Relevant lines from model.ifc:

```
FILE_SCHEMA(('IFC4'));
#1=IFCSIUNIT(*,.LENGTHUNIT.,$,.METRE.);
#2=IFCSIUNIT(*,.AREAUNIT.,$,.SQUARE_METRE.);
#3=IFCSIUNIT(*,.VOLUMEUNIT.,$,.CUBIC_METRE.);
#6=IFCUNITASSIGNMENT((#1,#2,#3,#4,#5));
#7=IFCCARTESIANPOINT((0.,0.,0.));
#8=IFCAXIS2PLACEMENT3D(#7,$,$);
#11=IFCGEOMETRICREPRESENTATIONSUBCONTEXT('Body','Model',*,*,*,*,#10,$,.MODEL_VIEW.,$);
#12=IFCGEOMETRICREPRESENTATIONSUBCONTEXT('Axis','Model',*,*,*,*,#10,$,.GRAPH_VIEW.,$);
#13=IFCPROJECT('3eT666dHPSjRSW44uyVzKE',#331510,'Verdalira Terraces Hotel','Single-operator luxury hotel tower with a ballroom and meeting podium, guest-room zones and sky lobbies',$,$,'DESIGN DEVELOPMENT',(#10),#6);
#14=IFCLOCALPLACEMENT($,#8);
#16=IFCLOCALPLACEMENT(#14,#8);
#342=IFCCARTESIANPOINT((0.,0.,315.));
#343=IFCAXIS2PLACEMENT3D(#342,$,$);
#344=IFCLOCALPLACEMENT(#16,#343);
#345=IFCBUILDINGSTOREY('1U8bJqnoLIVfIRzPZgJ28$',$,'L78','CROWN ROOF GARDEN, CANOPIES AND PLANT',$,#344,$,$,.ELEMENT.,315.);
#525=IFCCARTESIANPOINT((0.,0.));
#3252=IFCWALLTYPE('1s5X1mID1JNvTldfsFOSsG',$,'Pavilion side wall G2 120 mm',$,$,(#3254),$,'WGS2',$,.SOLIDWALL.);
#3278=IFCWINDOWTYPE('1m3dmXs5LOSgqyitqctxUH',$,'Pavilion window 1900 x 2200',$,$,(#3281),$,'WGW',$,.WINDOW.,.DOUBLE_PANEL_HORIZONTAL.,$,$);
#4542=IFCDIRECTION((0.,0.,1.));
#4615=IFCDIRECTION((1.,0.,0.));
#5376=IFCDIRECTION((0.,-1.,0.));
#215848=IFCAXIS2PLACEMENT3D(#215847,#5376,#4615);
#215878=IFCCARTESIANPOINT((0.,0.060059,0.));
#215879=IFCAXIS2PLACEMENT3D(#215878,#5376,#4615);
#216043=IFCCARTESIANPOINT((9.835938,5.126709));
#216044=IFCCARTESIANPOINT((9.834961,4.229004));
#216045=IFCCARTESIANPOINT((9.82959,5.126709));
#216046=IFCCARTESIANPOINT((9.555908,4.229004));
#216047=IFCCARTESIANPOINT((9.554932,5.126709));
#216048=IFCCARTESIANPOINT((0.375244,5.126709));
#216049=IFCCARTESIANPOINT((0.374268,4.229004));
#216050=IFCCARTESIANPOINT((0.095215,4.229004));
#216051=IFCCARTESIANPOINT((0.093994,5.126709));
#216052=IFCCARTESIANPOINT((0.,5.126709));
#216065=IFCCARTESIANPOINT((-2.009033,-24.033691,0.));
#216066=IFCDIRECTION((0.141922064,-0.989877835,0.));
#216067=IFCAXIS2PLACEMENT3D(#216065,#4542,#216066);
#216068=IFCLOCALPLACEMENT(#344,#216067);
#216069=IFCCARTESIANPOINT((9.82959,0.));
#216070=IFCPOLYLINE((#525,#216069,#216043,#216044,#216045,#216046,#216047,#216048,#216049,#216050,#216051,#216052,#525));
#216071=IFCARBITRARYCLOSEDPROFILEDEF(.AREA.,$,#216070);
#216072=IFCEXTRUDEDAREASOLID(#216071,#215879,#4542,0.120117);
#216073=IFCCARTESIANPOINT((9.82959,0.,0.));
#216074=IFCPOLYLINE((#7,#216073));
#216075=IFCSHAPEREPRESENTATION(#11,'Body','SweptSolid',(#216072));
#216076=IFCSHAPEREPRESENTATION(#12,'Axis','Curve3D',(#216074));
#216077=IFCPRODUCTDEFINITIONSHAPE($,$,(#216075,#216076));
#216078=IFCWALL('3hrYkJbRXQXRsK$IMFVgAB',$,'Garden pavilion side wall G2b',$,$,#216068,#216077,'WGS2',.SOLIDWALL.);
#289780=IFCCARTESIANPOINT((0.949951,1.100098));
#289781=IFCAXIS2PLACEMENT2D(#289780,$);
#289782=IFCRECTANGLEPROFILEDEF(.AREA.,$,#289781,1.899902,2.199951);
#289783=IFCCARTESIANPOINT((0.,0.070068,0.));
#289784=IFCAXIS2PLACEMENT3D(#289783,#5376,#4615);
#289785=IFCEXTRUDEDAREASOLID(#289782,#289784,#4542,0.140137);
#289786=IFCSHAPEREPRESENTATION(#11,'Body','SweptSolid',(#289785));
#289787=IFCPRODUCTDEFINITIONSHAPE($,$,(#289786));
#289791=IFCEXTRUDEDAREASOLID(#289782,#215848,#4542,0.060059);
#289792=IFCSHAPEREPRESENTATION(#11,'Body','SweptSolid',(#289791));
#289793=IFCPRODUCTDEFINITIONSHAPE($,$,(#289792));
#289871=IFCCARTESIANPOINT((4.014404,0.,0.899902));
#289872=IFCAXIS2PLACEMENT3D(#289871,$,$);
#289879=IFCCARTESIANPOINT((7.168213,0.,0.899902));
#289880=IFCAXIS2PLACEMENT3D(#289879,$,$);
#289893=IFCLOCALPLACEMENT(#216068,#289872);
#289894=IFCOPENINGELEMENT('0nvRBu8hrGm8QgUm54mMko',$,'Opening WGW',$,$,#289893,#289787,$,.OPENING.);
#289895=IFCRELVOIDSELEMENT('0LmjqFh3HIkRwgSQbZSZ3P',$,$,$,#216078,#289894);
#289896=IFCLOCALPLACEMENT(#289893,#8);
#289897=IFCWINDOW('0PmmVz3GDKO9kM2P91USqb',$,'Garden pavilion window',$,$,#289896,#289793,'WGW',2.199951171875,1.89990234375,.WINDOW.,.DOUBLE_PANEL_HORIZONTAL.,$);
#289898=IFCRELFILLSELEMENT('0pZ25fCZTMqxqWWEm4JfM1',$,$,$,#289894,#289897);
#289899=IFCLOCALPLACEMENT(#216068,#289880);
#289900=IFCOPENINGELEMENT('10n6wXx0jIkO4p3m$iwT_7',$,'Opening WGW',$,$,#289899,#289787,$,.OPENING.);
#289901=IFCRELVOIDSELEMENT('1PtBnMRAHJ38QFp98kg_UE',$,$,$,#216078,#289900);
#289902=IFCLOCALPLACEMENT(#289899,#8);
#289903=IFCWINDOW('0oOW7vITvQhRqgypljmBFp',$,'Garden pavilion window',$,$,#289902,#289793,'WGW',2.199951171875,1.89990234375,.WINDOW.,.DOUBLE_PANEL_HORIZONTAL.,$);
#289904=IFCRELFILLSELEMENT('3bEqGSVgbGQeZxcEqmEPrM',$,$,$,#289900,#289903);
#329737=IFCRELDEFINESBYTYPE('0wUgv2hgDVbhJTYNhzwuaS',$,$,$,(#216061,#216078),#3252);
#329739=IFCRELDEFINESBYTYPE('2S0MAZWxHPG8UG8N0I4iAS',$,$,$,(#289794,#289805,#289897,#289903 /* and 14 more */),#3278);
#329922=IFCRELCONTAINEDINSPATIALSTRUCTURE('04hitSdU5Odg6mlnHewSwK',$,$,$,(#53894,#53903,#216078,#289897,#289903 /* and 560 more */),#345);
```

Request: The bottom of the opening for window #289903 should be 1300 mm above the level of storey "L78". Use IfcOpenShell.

```python
import numpy as np
import ifcopenshell
import ifcopenshell.api.geometry
import ifcopenshell.geom
import ifcopenshell.util.element
import ifcopenshell.util.placement
import ifcopenshell.util.shape
import ifcopenshell.util.unit

model = ifcopenshell.open("model.ifc")
unit_scale = ifcopenshell.util.unit.calculate_unit_scale(model)

window = model.by_id(289903)
opening = window.FillsVoids[0].RelatingOpeningElement
storey = ifcopenshell.util.element.get_container(window, ifc_class="IfcBuildingStorey")
level = ifcopenshell.util.placement.get_local_placement(storey.ObjectPlacement)[2, 3]

# The opening's origin need not be at the sill, so measure its lowest point.
shape = ifcopenshell.geom.create_shape(ifcopenshell.geom.settings(), opening)
bottom = ifcopenshell.util.shape.get_shape_bottom_elevation(shape, shape.geometry) / unit_scale
dz = level + 1.3 / unit_scale - bottom

shift = np.array([0.0, 0.0, dz])
# The window is placed relative to its opening, so it follows when the opening moves.
matrix = ifcopenshell.util.placement.get_local_placement(opening.ObjectPlacement)
matrix[:3, 3] += shift
ifcopenshell.api.geometry.edit_object_placement(
    model, product=opening, matrix=matrix, is_si=False, should_transform_children=True
)

print(f"moved by {dz * unit_scale:+.3f} m")

model.write("model_rev.ifc")
```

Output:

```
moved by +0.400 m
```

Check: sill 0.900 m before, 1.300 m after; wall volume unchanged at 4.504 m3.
